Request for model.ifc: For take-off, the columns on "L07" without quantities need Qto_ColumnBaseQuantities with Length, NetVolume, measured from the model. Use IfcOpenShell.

First a look at what the model holds.

```python
import ifcopenshell
import ifcopenshell.util.element
import ifcopenshell.util.unit

model = ifcopenshell.open("model.ifc")
print(model.schema)
for unit_type in ("LENGTHUNIT", "AREAUNIT", "VOLUMEUNIT"):
    print(unit_type, ifcopenshell.util.unit.calculate_unit_scale(model, unit_type))
storey = next(s for s in model.by_type("IfcBuildingStorey") if s.Name == "L07")
columns = [e for e in ifcopenshell.util.element.get_decomposition(storey) if e.is_a("IfcColumn")]
for e in sorted(columns, key=lambda e: e.id()):
    print(e.id(), e.is_a(), e.Name, list(ifcopenshell.util.element.get_psets(e, qtos_only=True)), sep=" | ")
```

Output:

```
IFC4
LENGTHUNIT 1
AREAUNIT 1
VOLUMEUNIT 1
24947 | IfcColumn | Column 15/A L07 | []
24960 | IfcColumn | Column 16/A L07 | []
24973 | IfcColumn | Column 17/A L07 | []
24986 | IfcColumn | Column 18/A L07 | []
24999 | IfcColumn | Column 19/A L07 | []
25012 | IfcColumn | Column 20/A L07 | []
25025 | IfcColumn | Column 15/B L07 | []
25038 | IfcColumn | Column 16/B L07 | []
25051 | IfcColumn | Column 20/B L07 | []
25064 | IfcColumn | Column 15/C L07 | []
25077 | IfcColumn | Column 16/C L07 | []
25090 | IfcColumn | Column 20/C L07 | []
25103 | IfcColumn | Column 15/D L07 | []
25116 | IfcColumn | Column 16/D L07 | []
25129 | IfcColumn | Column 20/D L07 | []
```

```python
import ifcopenshell
import ifcopenshell.api.pset
import ifcopenshell.geom
import ifcopenshell.util.element
import ifcopenshell.util.shape
import ifcopenshell.util.unit

model = ifcopenshell.open("model.ifc")
unit_scale = ifcopenshell.util.unit.calculate_unit_scale(model)
volume_scale = ifcopenshell.util.unit.calculate_unit_scale(model, "VOLUMEUNIT")
settings = ifcopenshell.geom.settings()

storey = next(s for s in model.by_type("IfcBuildingStorey") if s.Name == "L07")
columns = [e for e in ifcopenshell.util.element.get_decomposition(storey) if e.is_a("IfcColumn")]

for e in sorted(columns, key=lambda e: e.id()):
    if ifcopenshell.util.element.get_psets(e, qtos_only=True, should_inherit=False):
        continue
    # Geometry comes back in metres, in the element's own axes.
    shape = ifcopenshell.geom.create_shape(settings, e)
    values = {
        "Length": ifcopenshell.util.shape.get_z(shape.geometry) / unit_scale,
        "NetVolume": ifcopenshell.util.shape.get_volume(shape.geometry) / volume_scale,
    }
    qto = ifcopenshell.api.pset.add_qto(model, product=e, name="Qto_ColumnBaseQuantities")
    ifcopenshell.api.pset.edit_qto(model, qto=qto, properties=values)
    print(e.id(), {k: round(v, 3) for k, v in values.items()})

model.write("model_rev.ifc")
```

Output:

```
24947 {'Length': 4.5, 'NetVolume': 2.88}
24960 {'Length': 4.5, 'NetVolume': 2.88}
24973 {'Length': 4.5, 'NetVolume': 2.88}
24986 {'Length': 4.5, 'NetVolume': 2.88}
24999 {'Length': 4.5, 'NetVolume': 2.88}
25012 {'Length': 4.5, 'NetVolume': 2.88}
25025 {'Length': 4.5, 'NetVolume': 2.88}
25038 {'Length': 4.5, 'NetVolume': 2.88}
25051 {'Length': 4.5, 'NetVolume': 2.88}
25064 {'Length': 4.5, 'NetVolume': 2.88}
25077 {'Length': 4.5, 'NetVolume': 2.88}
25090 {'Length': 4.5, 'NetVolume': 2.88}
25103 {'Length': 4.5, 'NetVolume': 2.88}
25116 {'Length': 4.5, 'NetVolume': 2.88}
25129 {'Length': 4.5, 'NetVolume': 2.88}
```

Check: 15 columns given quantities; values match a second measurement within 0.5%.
